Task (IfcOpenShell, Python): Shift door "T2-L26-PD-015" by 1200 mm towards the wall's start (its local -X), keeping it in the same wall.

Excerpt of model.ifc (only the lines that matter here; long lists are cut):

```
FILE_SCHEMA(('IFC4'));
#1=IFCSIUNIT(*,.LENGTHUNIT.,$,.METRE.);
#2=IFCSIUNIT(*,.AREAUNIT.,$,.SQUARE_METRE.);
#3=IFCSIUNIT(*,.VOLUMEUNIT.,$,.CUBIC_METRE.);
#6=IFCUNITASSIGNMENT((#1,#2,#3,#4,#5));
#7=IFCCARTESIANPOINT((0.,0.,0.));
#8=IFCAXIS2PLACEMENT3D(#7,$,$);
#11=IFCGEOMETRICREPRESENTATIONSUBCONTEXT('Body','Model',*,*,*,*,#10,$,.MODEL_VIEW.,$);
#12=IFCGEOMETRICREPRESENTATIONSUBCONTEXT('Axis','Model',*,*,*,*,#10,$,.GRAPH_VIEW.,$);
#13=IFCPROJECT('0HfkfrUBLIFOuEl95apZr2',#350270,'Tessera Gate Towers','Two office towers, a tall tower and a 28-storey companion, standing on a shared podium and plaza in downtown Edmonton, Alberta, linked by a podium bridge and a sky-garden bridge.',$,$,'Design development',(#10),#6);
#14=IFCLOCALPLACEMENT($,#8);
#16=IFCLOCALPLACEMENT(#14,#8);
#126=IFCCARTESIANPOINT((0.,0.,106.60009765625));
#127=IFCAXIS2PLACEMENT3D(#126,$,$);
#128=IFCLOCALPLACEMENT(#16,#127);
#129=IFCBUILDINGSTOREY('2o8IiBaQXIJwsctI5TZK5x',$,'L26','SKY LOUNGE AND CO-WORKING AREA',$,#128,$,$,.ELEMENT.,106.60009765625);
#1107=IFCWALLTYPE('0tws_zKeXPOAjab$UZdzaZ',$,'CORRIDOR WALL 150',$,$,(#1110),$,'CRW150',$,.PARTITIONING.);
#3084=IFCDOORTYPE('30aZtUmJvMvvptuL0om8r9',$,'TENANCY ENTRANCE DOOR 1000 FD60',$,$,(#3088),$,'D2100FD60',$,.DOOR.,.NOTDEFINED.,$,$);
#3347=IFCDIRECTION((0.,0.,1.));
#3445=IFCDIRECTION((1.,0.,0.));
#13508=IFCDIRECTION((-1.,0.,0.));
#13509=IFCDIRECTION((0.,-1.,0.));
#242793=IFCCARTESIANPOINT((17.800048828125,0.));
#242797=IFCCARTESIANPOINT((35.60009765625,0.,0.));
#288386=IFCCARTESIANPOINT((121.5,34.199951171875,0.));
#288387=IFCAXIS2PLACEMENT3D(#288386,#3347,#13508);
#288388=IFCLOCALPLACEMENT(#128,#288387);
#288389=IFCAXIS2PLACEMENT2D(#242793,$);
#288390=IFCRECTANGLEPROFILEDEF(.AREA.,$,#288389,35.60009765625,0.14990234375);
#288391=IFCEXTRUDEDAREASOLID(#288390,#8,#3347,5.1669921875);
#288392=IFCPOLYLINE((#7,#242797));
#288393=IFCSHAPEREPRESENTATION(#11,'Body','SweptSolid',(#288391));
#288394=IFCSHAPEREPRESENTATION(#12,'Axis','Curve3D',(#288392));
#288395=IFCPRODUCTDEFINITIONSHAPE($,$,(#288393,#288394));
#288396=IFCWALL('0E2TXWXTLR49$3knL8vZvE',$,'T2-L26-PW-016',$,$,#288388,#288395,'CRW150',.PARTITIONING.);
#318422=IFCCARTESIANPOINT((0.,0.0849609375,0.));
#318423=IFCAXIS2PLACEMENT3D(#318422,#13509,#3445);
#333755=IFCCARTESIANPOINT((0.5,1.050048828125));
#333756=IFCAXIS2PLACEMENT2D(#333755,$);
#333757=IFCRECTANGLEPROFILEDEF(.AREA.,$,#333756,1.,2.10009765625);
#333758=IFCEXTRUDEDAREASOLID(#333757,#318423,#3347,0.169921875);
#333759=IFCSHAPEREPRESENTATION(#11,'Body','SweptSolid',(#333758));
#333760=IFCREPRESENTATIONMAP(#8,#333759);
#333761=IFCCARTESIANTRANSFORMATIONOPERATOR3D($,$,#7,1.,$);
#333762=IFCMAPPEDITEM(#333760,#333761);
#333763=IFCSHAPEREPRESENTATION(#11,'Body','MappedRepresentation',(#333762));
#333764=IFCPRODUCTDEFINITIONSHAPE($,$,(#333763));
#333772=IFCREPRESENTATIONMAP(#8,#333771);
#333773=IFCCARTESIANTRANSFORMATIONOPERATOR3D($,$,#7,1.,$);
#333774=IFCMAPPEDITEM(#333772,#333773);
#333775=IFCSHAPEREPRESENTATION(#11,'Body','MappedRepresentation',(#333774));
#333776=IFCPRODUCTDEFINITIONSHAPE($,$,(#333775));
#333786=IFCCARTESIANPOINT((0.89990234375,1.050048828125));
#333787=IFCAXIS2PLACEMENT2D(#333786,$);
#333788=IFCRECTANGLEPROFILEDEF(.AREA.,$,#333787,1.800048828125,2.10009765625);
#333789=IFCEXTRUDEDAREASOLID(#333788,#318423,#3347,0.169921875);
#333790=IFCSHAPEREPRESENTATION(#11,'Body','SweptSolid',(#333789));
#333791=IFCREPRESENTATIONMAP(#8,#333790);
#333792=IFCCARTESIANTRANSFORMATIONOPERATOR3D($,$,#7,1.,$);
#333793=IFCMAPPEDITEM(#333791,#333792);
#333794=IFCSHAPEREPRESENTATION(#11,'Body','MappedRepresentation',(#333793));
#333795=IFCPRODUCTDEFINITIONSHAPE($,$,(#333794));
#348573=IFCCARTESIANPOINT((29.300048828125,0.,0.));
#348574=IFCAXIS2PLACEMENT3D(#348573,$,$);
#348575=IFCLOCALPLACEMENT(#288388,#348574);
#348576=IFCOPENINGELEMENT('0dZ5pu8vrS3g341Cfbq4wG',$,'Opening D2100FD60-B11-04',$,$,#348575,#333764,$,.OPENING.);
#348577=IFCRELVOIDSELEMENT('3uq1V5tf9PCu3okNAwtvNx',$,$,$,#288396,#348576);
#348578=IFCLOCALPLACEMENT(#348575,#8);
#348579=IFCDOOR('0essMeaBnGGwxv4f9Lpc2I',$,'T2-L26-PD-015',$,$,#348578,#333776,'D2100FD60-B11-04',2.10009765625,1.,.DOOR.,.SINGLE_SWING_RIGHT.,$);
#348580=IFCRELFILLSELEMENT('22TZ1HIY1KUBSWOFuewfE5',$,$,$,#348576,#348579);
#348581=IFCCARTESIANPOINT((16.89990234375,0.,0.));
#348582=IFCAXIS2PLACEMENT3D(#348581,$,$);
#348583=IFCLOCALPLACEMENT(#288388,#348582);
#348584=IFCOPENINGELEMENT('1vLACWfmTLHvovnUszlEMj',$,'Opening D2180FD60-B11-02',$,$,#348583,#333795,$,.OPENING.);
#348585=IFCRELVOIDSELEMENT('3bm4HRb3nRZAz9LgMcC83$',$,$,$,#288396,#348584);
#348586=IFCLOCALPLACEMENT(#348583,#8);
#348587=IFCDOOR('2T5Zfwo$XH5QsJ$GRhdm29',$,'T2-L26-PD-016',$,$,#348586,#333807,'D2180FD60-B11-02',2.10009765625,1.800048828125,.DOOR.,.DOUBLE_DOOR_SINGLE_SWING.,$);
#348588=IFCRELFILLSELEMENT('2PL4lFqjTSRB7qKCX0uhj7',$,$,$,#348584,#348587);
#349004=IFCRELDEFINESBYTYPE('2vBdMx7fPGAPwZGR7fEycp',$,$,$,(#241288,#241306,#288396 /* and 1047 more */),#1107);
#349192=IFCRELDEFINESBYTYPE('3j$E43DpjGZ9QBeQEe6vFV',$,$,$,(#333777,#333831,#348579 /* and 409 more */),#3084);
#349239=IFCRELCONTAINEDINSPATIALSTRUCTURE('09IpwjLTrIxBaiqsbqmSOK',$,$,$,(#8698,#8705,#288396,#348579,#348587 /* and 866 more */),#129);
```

```python
import ifcopenshell
import ifcopenshell.api.geometry
import ifcopenshell.util.placement

model = ifcopenshell.open("model.ifc")

door = model.by_id(348579)
opening = door.FillsVoids[0].RelatingOpeningElement
wall = opening.VoidsElements[0].RelatingBuildingElement

wall_matrix = ifcopenshell.util.placement.get_local_placement(wall.ObjectPlacement)
shift = wall_matrix[:3, 0] * -1.2
before = ifcopenshell.util.placement.get_local_placement(door.ObjectPlacement)[:3, 3].copy()

# The door is placed relative to its opening, so it follows when the opening moves.
matrix = ifcopenshell.util.placement.get_local_placement(opening.ObjectPlacement)
matrix[:3, 3] += shift
ifcopenshell.api.geometry.edit_object_placement(
    model, product=opening, matrix=matrix, is_si=False, should_transform_children=True
)

after = ifcopenshell.util.placement.get_local_placement(door.ObjectPlacement)[:3, 3]
print("door moved by", (after - before).round(3) + 0.0)

model.write("model-out.ifc")
```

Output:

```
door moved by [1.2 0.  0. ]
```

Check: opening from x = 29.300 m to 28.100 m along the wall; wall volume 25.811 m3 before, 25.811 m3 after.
